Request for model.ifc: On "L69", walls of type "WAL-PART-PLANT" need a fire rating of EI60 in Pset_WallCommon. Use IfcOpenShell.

First a look at what the model holds.

```python
import ifcopenshell
import ifcopenshell.util.element

model = ifcopenshell.open("model.ifc")
print(model.schema)
storey = next(s for s in model.by_type("IfcBuildingStorey") if s.Name == "L69")
walls = [e for e in ifcopenshell.util.element.get_decomposition(storey) if e.is_a("IfcWall")]
seen = {}
for e in walls:
    element_type = ifcopenshell.util.element.get_type(e)
    key = (element_type.Name if element_type != e and element_type else None, ifcopenshell.util.element.get_pset(e, "Pset_WallCommon", "FireRating"))
    seen[key] = seen.get(key, 0) + 1
for (name, value), count in sorted(seen.items(), key=str):
    print(count, "x", name, "|", value)
```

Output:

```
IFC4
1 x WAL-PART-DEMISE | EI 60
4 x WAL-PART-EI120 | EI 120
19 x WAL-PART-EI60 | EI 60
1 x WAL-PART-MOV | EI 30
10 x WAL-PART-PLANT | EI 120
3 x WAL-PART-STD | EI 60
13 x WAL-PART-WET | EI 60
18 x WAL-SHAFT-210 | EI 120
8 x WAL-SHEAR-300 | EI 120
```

```python
import ifcopenshell
import ifcopenshell.api.pset
import ifcopenshell.util.element

model = ifcopenshell.open("model.ifc")

storey = next(s for s in model.by_type("IfcBuildingStorey") if s.Name == "L69")
walls = [e for e in ifcopenshell.util.element.get_decomposition(storey) if e.is_a("IfcWall")]

count = 0
for e in walls:
    element_type = ifcopenshell.util.element.get_type(e)
    if element_type in (None, e) or element_type.Name != "WAL-PART-PLANT":
        continue
    # add_pset returns the element's existing set when there is one.
    pset = ifcopenshell.api.pset.add_pset(model, product=e, name="Pset_WallCommon")
    ifcopenshell.api.pset.edit_pset(model, pset=pset, properties={"FireRating": "EI60"})
    count += 1

print(count, "walls updated")

model.write("model_rev.ifc")
```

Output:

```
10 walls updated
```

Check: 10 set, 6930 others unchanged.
